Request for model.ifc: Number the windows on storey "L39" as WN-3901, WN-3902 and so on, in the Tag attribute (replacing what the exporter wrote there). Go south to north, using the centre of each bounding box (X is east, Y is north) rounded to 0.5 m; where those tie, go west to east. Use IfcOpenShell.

First a look at what the model holds.

```python
import ifcopenshell
import ifcopenshell.util.element
import ifcopenshell.util.placement

model = ifcopenshell.open("model.ifc")
print(model.schema)
storey = next(s for s in model.by_type("IfcBuildingStorey") if s.Name == "L39")
windows = [e for e in ifcopenshell.util.element.get_decomposition(storey) if e.is_a("IfcWindow")]
for e in sorted(windows, key=lambda e: e.id()):
    origin = ifcopenshell.util.placement.get_local_placement(e.ObjectPlacement)[:3, 3]
    print(e.id(), e.Tag, e.Name, origin.round(2) + 0.0, sep=" | ")
```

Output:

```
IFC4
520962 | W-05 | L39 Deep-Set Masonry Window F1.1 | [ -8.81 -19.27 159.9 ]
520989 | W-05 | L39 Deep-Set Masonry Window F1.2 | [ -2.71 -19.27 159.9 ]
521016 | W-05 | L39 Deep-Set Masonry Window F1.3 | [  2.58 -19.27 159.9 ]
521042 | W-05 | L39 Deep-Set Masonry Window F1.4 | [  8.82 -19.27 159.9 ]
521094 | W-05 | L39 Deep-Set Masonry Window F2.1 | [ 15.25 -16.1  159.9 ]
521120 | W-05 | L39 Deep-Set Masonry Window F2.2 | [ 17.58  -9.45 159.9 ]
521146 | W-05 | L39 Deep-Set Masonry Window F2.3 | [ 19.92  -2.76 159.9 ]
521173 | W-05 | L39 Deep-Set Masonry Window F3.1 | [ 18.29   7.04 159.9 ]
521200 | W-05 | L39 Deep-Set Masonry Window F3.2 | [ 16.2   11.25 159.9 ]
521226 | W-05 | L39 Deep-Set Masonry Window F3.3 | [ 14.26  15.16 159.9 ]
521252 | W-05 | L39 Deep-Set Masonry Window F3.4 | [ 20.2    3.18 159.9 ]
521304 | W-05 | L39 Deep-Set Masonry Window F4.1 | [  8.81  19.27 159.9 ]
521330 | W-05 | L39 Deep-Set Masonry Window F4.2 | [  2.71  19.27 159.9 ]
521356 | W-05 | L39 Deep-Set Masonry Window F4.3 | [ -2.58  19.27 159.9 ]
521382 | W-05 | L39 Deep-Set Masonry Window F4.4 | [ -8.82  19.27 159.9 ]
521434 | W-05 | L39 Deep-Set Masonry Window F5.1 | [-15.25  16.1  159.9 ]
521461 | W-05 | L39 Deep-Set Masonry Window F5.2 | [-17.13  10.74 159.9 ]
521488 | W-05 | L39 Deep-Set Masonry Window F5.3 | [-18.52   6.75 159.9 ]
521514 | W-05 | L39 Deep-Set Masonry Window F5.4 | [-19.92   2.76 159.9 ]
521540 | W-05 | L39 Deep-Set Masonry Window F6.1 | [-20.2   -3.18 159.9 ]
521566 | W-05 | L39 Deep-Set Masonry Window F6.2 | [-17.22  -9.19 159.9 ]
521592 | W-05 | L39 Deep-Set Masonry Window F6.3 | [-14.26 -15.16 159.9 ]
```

```python
import ifcopenshell
import ifcopenshell.geom
import ifcopenshell.util.element
import ifcopenshell.util.shape

model = ifcopenshell.open("model.ifc")
settings = ifcopenshell.geom.settings()
settings.set("use-world-coords", True)


def centre(element):
    shape = ifcopenshell.geom.create_shape(settings, element)
    return ifcopenshell.util.shape.get_bbox_centroid(shape.geometry)


storey = next(s for s in model.by_type("IfcBuildingStorey") if s.Name == "L39")
windows = [e for e in ifcopenshell.util.element.get_decomposition(storey) if e.is_a("IfcWindow")]

# Insertion points can sit at a corner or the storey origin, so sort by the geometry (in metres).
centres = {e: centre(e) for e in windows}
windows.sort(key=lambda e: (round(centres[e][1] / 0.5), centres[e][0]))

for i, e in enumerate(windows, start=1):
    number = f"WN-39{i:02d}"
    e.Tag = number
    print(e.id(), number)

model.write("model_updated.ifc")
```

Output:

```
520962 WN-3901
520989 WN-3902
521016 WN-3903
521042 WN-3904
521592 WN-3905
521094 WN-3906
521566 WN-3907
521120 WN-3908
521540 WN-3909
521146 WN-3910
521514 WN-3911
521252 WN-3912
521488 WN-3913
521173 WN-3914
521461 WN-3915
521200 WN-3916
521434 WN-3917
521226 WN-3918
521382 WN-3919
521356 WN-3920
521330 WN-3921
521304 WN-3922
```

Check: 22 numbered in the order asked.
